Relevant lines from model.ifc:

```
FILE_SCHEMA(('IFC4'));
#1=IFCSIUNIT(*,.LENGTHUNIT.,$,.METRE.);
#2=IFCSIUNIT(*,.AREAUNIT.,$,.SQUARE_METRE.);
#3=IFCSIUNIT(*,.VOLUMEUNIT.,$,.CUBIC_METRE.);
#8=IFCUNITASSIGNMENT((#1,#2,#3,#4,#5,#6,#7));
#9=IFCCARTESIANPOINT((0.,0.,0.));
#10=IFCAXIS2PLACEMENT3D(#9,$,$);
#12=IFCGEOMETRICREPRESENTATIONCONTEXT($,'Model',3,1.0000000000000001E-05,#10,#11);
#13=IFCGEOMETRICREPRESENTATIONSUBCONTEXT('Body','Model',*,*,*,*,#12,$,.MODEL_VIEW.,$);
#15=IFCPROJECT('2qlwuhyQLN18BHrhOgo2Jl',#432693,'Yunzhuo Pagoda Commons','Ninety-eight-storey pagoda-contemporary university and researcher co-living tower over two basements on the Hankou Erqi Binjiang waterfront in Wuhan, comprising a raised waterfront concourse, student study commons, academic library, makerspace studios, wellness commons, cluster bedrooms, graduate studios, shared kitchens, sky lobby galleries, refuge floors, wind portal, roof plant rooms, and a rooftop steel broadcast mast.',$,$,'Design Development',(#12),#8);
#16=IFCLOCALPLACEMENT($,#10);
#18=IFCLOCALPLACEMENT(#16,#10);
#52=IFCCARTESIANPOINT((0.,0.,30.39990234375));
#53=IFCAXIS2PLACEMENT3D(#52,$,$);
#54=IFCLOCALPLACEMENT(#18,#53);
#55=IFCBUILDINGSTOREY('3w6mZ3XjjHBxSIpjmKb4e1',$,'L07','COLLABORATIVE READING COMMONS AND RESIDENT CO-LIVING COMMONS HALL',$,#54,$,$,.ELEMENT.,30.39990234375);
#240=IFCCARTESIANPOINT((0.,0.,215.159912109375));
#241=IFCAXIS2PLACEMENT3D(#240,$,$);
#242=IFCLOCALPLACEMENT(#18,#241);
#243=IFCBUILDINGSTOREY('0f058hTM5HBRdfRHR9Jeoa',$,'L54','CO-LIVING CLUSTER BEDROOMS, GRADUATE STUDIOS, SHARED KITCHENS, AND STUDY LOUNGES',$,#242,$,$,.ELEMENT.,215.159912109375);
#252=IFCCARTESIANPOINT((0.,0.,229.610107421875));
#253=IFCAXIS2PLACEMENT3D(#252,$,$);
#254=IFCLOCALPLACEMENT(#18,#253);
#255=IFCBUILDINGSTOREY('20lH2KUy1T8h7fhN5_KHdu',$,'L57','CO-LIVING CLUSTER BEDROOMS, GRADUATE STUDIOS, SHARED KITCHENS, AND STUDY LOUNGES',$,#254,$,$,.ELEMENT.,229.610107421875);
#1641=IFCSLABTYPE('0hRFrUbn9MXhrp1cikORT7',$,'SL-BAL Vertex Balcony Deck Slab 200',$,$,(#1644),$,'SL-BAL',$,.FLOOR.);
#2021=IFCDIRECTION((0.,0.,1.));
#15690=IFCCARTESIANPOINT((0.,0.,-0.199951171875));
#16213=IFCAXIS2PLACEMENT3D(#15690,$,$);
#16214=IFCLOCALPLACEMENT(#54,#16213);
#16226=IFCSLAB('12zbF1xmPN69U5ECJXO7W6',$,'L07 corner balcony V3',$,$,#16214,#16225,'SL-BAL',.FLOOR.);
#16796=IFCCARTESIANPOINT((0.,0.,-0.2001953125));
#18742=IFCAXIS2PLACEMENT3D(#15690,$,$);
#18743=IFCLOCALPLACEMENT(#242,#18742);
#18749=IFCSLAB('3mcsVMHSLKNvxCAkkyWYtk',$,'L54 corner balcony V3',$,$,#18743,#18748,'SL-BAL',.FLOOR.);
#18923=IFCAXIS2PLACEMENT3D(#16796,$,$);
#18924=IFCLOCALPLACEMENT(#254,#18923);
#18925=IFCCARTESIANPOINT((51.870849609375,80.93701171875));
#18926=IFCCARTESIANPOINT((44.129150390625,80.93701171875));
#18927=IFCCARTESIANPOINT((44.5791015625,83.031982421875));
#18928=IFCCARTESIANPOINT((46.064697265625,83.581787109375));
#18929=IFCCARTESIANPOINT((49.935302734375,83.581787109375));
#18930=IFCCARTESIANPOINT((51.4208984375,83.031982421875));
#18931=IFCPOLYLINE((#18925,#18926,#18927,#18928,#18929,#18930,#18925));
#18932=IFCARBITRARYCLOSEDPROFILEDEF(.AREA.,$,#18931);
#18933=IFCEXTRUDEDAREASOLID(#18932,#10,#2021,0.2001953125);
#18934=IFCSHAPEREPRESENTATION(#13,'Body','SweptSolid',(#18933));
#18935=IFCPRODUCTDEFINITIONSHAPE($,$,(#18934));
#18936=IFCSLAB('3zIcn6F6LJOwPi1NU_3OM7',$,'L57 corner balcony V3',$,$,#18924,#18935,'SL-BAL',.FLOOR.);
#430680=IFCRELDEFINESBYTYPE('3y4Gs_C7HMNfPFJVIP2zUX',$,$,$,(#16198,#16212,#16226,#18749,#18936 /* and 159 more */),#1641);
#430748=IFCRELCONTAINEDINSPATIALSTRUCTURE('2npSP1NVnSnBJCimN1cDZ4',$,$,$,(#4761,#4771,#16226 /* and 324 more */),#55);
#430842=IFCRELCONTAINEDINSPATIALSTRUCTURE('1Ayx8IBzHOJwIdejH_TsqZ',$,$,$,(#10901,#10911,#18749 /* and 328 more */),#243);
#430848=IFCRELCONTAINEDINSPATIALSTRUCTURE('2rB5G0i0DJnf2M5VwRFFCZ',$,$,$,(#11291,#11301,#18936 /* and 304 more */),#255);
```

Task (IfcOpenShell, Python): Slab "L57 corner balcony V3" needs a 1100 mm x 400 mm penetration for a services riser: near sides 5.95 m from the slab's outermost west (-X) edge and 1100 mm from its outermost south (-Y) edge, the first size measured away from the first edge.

```python
import numpy as np
import ifcopenshell
import ifcopenshell.api.feature
import ifcopenshell.api.geometry
import ifcopenshell.api.root
import ifcopenshell.geom
import ifcopenshell.util.placement
import ifcopenshell.util.representation
import ifcopenshell.util.shape
import ifcopenshell.util.unit

model = ifcopenshell.open("model.ifc")
unit_scale = ifcopenshell.util.unit.calculate_unit_scale(model)
settings = ifcopenshell.geom.settings()


def volume(element):
    """Net volume in cubic metres, openings subtracted."""
    shape = ifcopenshell.geom.create_shape(settings, element)
    return ifcopenshell.util.shape.get_volume(shape.geometry)


slab = model.by_id(18936)
before = volume(slab)

# Extent in the slab's own axes, in metres. The edges named are its -X and -Y sides.
slab_shape = ifcopenshell.geom.create_shape(settings, slab)
vertices = ifcopenshell.util.shape.get_vertices(slab_shape.geometry)
x_min, y_min, bottom = vertices.min(axis=0)
top = vertices[:, 2].max()

opening = ifcopenshell.api.root.create_entity(model, ifc_class="IfcOpeningElement", name="Services riser opening", predefined_type="OPENING")
context = ifcopenshell.util.representation.get_context(model, "Model", "Body", "MODEL_VIEW")
width, depth = 1.1, 0.4
outline = [(0.0, 0.0), (width, 0.0), (width, depth), (0.0, depth), (0.0, 0.0)]
# Overshoot both faces by 50 mm so the cut is clean.
shape = ifcopenshell.api.geometry.add_slab_representation(
    model, context=context, depth=top - bottom + 0.1, polyline=outline
)
ifcopenshell.api.geometry.assign_representation(model, product=opening, representation=shape)

matrix = ifcopenshell.util.placement.get_local_placement(slab.ObjectPlacement)
matrix[:, 3] = matrix @ np.append(np.array([x_min + 5.95, y_min + 1.1, bottom - 0.05]) / unit_scale, 1.0)
ifcopenshell.api.geometry.edit_object_placement(model, product=opening, matrix=matrix, is_si=False)
ifcopenshell.api.feature.add_feature(model, feature=opening, element=slab)

after = volume(slab)

print(f"slab volume {before:.3f} -> {after:.3f} m3")

model.write("model_edited.ifc")
```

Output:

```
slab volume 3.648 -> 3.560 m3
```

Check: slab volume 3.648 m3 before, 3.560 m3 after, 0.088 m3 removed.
